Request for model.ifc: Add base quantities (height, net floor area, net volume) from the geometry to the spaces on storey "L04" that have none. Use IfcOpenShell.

First a look at what the model holds.

```python
import ifcopenshell
import ifcopenshell.util.element
import ifcopenshell.util.unit

model = ifcopenshell.open("model.ifc")
print(model.schema)
for unit_type in ("LENGTHUNIT", "AREAUNIT", "VOLUMEUNIT"):
    print(unit_type, ifcopenshell.util.unit.calculate_unit_scale(model, unit_type))
storey = next(s for s in model.by_type("IfcBuildingStorey") if s.Name == "L04")
spaces = [e for e in ifcopenshell.util.element.get_decomposition(storey) if e.is_a("IfcSpace")]
for e in sorted(spaces, key=lambda e: e.id()):
    print(e.id(), e.is_a(), e.Name, list(ifcopenshell.util.element.get_psets(e, qtos_only=True)), sep=" | ")
```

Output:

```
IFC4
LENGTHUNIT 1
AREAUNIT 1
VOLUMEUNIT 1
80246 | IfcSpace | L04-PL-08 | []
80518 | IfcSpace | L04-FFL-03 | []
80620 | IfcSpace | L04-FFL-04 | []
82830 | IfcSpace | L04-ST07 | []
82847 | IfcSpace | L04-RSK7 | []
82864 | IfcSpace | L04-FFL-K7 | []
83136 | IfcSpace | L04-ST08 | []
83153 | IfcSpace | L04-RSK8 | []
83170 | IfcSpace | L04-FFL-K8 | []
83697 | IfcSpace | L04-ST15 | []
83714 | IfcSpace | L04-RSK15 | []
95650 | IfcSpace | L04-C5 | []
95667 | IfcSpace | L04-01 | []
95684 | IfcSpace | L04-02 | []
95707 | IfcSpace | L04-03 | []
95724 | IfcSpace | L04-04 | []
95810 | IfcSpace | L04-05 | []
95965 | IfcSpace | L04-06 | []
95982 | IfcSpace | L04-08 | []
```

```python
import ifcopenshell
import ifcopenshell.api.pset
import ifcopenshell.geom
import ifcopenshell.util.element
import ifcopenshell.util.shape
import ifcopenshell.util.unit

model = ifcopenshell.open("model.ifc")
unit_scale = ifcopenshell.util.unit.calculate_unit_scale(model)
area_scale = ifcopenshell.util.unit.calculate_unit_scale(model, "AREAUNIT")
volume_scale = ifcopenshell.util.unit.calculate_unit_scale(model, "VOLUMEUNIT")
settings = ifcopenshell.geom.settings()

storey = next(s for s in model.by_type("IfcBuildingStorey") if s.Name == "L04")
spaces = [e for e in ifcopenshell.util.element.get_decomposition(storey) if e.is_a("IfcSpace")]

for e in sorted(spaces, key=lambda e: e.id()):
    if ifcopenshell.util.element.get_psets(e, qtos_only=True, should_inherit=False):
        continue
    # Geometry comes back in metres, in the element's own axes.
    shape = ifcopenshell.geom.create_shape(settings, e)
    values = {
        "Height": ifcopenshell.util.shape.get_z(shape.geometry) / unit_scale,
        "NetFloorArea": ifcopenshell.util.shape.get_footprint_area(shape.geometry) / area_scale,
        "NetVolume": ifcopenshell.util.shape.get_volume(shape.geometry) / volume_scale,
    }
    qto = ifcopenshell.api.pset.add_qto(model, product=e, name="Qto_SpaceBaseQuantities")
    ifcopenshell.api.pset.edit_qto(model, qto=qto, properties=values)
    print(e.id(), {k: round(v, 3) for k, v in values.items()})

model.write("model_edited.ifc")
```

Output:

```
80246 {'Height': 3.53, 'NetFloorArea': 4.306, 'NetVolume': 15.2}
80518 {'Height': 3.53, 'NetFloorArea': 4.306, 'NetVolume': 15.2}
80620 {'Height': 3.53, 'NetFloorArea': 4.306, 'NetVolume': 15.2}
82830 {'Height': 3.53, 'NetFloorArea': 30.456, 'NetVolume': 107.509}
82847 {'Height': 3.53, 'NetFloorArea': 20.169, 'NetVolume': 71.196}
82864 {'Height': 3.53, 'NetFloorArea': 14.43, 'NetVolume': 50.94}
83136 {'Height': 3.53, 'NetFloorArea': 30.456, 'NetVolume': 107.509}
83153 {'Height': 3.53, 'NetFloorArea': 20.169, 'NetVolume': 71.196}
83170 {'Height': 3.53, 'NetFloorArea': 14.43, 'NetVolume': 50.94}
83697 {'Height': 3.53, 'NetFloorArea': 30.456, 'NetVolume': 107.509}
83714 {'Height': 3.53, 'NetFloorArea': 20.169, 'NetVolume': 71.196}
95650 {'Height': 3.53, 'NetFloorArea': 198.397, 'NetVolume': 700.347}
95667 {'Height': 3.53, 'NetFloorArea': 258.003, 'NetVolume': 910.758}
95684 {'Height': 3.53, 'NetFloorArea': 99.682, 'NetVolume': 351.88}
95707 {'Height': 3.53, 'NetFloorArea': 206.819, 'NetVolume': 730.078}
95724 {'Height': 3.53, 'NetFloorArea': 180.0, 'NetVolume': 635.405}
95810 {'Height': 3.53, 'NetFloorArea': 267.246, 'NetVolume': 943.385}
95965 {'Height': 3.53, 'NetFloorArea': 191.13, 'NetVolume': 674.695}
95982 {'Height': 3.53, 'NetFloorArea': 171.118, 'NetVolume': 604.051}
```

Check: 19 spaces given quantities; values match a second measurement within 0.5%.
